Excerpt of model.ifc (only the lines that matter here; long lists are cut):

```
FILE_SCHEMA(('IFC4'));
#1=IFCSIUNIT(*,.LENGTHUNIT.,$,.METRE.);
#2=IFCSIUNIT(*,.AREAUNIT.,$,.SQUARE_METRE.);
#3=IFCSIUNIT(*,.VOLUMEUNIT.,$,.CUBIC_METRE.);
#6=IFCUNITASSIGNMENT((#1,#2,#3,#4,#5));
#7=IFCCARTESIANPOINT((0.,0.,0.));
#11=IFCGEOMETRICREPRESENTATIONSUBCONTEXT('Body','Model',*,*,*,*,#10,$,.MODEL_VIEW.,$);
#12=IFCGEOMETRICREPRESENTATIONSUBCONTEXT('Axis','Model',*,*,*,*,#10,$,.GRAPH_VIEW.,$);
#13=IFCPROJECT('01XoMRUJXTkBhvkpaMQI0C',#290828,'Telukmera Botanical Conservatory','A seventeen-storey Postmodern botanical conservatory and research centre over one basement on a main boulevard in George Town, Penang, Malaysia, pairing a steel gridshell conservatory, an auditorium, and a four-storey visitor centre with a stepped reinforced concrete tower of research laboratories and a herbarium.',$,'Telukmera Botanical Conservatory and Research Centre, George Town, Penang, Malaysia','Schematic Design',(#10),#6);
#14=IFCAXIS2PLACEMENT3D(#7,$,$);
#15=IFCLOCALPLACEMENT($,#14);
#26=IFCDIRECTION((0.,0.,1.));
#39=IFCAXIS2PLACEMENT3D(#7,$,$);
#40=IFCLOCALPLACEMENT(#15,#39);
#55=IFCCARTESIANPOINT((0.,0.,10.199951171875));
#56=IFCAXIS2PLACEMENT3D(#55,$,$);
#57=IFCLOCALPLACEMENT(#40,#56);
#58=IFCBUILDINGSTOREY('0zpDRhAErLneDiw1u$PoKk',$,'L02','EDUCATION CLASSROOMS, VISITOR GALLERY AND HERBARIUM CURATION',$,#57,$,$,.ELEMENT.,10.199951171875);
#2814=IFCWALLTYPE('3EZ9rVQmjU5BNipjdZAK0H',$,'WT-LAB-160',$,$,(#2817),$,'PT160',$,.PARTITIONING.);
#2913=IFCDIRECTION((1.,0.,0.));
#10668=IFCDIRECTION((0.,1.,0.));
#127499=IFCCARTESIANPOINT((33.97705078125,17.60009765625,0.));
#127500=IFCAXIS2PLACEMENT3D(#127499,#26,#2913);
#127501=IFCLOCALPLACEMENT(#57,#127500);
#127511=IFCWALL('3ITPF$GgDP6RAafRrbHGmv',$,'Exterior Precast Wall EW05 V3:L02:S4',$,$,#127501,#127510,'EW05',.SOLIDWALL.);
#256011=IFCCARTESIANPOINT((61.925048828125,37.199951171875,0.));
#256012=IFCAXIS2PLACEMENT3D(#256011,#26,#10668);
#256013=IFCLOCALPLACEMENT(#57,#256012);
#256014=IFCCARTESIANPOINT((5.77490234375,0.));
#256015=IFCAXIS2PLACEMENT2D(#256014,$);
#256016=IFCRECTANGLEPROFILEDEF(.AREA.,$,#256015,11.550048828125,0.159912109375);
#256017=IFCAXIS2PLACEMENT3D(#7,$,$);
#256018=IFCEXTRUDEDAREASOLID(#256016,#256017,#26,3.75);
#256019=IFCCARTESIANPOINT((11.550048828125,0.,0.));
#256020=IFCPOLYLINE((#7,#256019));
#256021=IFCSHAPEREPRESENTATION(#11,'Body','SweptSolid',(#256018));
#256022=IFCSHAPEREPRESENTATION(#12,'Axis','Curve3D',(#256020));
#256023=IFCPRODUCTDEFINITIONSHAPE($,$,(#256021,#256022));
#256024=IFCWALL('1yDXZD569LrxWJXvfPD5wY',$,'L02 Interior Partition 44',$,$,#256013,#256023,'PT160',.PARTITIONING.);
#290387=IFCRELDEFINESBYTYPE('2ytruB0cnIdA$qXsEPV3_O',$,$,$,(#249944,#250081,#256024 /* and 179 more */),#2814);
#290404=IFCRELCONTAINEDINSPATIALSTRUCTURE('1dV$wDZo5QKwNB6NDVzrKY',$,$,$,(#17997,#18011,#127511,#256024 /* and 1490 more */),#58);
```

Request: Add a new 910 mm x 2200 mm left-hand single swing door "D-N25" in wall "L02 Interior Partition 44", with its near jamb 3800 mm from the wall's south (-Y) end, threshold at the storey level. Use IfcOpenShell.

```python
import numpy as np
import ifcopenshell
import ifcopenshell.api.feature
import ifcopenshell.api.geometry
import ifcopenshell.api.root
import ifcopenshell.api.spatial
import ifcopenshell.geom
import ifcopenshell.util.element
import ifcopenshell.util.placement
import ifcopenshell.util.representation
import ifcopenshell.util.shape
import ifcopenshell.util.unit

model = ifcopenshell.open("model.ifc")
unit_scale = ifcopenshell.util.unit.calculate_unit_scale(model)
settings = ifcopenshell.geom.settings()


def volume(element):
    """Net volume in cubic metres, openings subtracted."""
    shape = ifcopenshell.geom.create_shape(settings, element)
    return ifcopenshell.util.shape.get_volume(shape.geometry)


wall = model.by_id(256024)
storey = ifcopenshell.util.element.get_container(wall, ifc_class="IfcBuildingStorey")
context = ifcopenshell.util.representation.get_context(model, "Model", "Body", "MODEL_VIEW")
before = volume(wall)

width, height, from_end, sill = 0.91, 2.2, 3.8, 0.0  # metres

# The wall runs along its own X axis, and the end named is its -X end.
wall_shape = ifcopenshell.geom.create_shape(settings, wall)
x, y, z = ifcopenshell.util.shape.get_vertices(wall_shape.geometry).T
start = x.min() + from_end
face, thickness = float(y.min()), float(y.max() - y.min())
wall_matrix = ifcopenshell.util.placement.get_local_placement(wall.ObjectPlacement)
level = ifcopenshell.util.placement.get_local_placement(storey.ObjectPlacement)[2, 3]


def in_wall(x, y):
    """Placement at x, y metres in the wall's axes, at sill height."""
    matrix = wall_matrix.copy()
    matrix[:, 3] = wall_matrix @ np.array([x / unit_scale, y / unit_scale, 0.0, 1.0])
    matrix[2, 3] = level + sill / unit_scale
    return matrix


# Opening: a box that overshoots both wall faces by 50 mm.
opening = ifcopenshell.api.root.create_entity(model, ifc_class="IfcOpeningElement", predefined_type="OPENING")
box = ifcopenshell.api.geometry.add_wall_representation(
    model, context=context, length=width, height=height, thickness=thickness + 0.1
)
ifcopenshell.api.geometry.assign_representation(model, product=opening, representation=box)
ifcopenshell.api.geometry.edit_object_placement(model, product=opening, matrix=in_wall(start, face - 0.05), is_si=False)
ifcopenshell.api.feature.add_feature(model, feature=opening, element=wall)

door = ifcopenshell.api.root.create_entity(model, ifc_class="IfcDoor", name="D-N25", predefined_type="DOOR")
door.OverallWidth, door.OverallHeight = width / unit_scale, height / unit_scale
door.OperationType = "SINGLE_SWING_LEFT"
body = ifcopenshell.api.geometry.add_door_representation(
    model,
    context=context,
    overall_width=door.OverallWidth,
    overall_height=door.OverallHeight,
    operation_type="SINGLE_SWING_LEFT",
    lining_properties={"LiningDepth": thickness / unit_scale, "ThresholdDepth": thickness / unit_scale},
)
ifcopenshell.api.geometry.assign_representation(model, product=door, representation=body)
ifcopenshell.api.spatial.assign_container(model, products=[door], relating_structure=storey)
ifcopenshell.api.feature.add_filling(model, opening=opening, element=door)

# The lining spans the wall, so the door starts at the wall face.
ifcopenshell.api.geometry.edit_object_placement(model, product=door, matrix=in_wall(start, face), is_si=False)

after = volume(wall)

print(f"wall volume {before:.3f} -> {after:.3f} m3")

model.write("model_v2.ifc")
```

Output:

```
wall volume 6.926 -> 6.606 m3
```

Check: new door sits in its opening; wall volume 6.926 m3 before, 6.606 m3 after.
